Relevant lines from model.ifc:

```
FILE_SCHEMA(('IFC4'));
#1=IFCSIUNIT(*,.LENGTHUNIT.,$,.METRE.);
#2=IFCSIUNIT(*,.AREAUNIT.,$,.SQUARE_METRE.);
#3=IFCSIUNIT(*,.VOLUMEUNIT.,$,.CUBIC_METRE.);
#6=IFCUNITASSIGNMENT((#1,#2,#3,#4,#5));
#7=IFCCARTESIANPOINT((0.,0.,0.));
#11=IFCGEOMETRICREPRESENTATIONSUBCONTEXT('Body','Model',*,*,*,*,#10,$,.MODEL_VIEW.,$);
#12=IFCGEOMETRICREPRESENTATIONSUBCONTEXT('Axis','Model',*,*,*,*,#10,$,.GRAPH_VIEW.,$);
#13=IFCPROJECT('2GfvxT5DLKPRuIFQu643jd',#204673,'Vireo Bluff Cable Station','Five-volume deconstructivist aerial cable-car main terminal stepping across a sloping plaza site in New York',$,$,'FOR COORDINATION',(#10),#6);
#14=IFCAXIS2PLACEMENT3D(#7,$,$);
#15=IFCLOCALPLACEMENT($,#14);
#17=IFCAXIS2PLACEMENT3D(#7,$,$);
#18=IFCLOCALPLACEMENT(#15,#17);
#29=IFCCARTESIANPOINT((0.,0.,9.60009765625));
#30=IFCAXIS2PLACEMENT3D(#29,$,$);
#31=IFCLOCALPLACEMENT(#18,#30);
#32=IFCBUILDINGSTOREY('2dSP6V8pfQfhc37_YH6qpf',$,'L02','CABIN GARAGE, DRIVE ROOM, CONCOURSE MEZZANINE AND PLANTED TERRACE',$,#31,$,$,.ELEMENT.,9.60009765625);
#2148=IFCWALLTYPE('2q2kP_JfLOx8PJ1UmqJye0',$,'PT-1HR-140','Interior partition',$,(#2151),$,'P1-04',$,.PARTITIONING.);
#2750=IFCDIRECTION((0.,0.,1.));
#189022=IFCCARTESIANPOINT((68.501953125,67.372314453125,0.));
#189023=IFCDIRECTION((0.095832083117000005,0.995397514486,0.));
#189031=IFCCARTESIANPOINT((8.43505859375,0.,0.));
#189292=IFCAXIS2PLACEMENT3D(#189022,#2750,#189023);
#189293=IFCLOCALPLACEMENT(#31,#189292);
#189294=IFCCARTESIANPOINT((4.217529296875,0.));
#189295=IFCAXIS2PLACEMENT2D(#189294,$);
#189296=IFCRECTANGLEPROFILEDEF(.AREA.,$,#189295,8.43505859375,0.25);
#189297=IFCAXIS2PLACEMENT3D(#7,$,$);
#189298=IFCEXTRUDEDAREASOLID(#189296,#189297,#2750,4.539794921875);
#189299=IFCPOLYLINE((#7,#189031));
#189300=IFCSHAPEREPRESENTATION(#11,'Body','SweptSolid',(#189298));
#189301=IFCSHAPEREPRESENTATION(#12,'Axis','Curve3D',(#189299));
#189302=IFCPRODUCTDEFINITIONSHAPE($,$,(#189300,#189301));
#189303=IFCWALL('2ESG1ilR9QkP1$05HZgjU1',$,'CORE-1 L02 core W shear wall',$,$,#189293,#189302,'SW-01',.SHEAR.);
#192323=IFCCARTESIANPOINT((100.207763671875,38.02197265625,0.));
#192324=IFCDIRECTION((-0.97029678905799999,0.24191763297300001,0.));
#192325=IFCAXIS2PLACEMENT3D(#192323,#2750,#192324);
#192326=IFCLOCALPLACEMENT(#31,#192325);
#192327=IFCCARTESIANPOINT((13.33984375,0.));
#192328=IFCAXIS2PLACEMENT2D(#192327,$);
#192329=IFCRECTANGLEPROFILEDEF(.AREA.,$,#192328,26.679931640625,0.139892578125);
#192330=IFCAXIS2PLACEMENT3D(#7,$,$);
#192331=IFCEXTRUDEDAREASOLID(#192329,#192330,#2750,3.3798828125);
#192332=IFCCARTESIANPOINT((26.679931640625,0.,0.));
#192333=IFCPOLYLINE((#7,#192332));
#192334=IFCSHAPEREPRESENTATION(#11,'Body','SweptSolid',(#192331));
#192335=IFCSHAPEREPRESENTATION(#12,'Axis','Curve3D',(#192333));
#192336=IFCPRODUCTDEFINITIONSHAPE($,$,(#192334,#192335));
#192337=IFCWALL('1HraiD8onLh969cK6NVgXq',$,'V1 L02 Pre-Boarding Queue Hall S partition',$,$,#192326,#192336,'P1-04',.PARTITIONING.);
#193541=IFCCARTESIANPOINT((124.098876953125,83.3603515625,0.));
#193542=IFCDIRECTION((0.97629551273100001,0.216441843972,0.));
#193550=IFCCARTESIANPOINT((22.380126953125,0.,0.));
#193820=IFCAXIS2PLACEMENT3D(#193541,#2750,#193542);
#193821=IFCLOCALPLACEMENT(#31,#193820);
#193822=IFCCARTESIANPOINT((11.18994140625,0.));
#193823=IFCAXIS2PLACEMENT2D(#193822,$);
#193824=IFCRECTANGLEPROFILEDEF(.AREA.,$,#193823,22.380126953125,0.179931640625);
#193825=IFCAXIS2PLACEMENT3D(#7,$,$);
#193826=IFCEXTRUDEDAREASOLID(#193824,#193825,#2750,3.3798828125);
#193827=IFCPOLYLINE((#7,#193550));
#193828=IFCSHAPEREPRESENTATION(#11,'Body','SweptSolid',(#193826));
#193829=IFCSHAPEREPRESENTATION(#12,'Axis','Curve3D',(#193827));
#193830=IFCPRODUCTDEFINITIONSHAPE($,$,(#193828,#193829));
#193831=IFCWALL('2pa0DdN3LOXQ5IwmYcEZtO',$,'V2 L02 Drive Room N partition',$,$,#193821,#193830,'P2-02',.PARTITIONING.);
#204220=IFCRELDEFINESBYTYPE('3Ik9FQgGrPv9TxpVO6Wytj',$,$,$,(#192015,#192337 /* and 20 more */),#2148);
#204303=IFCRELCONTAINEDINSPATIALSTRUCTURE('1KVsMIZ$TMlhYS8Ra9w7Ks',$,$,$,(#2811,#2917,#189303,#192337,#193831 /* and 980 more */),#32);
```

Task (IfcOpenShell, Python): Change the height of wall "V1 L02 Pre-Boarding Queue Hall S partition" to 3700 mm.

```python
import ifcopenshell
import ifcopenshell.geom
import ifcopenshell.util.representation
import ifcopenshell.util.shape

model = ifcopenshell.open("model.ifc")
settings = ifcopenshell.geom.settings()


def volume(element):
    """Net volume in cubic metres, openings subtracted."""
    shape = ifcopenshell.geom.create_shape(settings, element)
    return ifcopenshell.util.shape.get_volume(shape.geometry)


wall = model.by_guid("1HraiD8onLh969cK6NVgXq")
before = volume(wall)

body = ifcopenshell.util.representation.get_representation(wall, "Model", "Body")
solid = body.Items[0]
old_height = solid.Depth
solid.Depth = 3.7
after = volume(wall)

print(f"height {old_height:g} -> {solid.Depth:g}, volume {before:.3f} -> {after:.3f} m3")

model.write("model-out.ifc")
```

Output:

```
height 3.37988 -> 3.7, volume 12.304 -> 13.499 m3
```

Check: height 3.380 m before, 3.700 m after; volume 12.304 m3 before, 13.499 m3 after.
